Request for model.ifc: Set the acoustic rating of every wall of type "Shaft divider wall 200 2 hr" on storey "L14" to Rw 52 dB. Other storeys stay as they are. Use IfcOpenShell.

First a look at what the model holds.

```python
import ifcopenshell
import ifcopenshell.util.element

model = ifcopenshell.open("model.ifc")
print(model.schema)
storey = next(s for s in model.by_type("IfcBuildingStorey") if s.Name == "L14")
walls = [e for e in ifcopenshell.util.element.get_decomposition(storey) if e.is_a("IfcWall")]
seen = {}
for e in walls:
    element_type = ifcopenshell.util.element.get_type(e)
    key = (element_type.Name if element_type != e and element_type else None, ifcopenshell.util.element.get_pset(e, "Pset_WallCommon", "AcousticRating"))
    seen[key] = seen.get(key, 0) + 1
for (name, value), count in sorted(seen.items(), key=str):
    print(count, "x", name, "|", value)
```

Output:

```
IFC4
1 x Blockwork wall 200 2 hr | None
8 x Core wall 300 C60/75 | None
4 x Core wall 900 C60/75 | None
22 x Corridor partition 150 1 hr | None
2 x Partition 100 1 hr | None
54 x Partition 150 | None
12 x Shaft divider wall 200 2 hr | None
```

```python
import ifcopenshell
import ifcopenshell.api.pset
import ifcopenshell.util.element

model = ifcopenshell.open("model.ifc")

storey = next(s for s in model.by_type("IfcBuildingStorey") if s.Name == "L14")
walls = [e for e in ifcopenshell.util.element.get_decomposition(storey) if e.is_a("IfcWall")]

count = 0
for e in walls:
    element_type = ifcopenshell.util.element.get_type(e)
    if element_type in (None, e) or element_type.Name != "Shaft divider wall 200 2 hr":
        continue
    found = ifcopenshell.util.element.get_pset(e, "Pset_WallCommon", should_inherit=False)
    if found:
        pset = model.by_id(found["id"])
        if len(ifcopenshell.util.element.get_elements_by_pset(pset)) > 1:
            pset = ifcopenshell.api.pset.unshare_pset(model, products=[e], pset=pset)[0]
    else:
        pset = ifcopenshell.api.pset.add_pset(model, product=e, name="Pset_WallCommon")
    ifcopenshell.api.pset.edit_pset(model, pset=pset, properties={"AcousticRating": "Rw 52 dB"})
    count += 1

print(count, "walls updated")

model.write("model_edited.ifc")
```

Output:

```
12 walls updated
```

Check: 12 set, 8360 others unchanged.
